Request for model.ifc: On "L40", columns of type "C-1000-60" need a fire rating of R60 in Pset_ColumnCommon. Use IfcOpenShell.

First a look at what the model holds.

```python
import ifcopenshell
import ifcopenshell.util.element

model = ifcopenshell.open("model.ifc")
print(model.schema)
storey = next(s for s in model.by_type("IfcBuildingStorey") if s.Name == "L40")
columns = [e for e in ifcopenshell.util.element.get_decomposition(storey) if e.is_a("IfcColumn")]
seen = {}
for e in columns:
    element_type = ifcopenshell.util.element.get_type(e)
    key = (element_type.Name if element_type != e and element_type else None, ifcopenshell.util.element.get_pset(e, "Pset_ColumnCommon", "FireRating"))
    seen[key] = seen.get(key, 0) + 1
for (name, value), count in sorted(seen.items(), key=str):
    print(count, "x", name, "|", value)
```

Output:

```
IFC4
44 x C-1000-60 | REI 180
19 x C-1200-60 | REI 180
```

```python
import ifcopenshell
import ifcopenshell.api.pset
import ifcopenshell.util.element

model = ifcopenshell.open("model.ifc")

storey = next(s for s in model.by_type("IfcBuildingStorey") if s.Name == "L40")
columns = [e for e in ifcopenshell.util.element.get_decomposition(storey) if e.is_a("IfcColumn")]

count = 0
for e in columns:
    element_type = ifcopenshell.util.element.get_type(e)
    if element_type in (None, e) or element_type.Name != "C-1000-60":
        continue
    found = ifcopenshell.util.element.get_pset(e, "Pset_ColumnCommon", should_inherit=False)
    if found:
        pset = model.by_id(found["id"])
        if len(ifcopenshell.util.element.get_elements_by_pset(pset)) > 1:
            pset = ifcopenshell.api.pset.unshare_pset(model, products=[e], pset=pset)[0]
    else:
        pset = ifcopenshell.api.pset.add_pset(model, product=e, name="Pset_ColumnCommon")
    ifcopenshell.api.pset.edit_pset(model, pset=pset, properties={"FireRating": "R60"})
    count += 1

print(count, "columns updated")

model.write("model_rev.ifc")
```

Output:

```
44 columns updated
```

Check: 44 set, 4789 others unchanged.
